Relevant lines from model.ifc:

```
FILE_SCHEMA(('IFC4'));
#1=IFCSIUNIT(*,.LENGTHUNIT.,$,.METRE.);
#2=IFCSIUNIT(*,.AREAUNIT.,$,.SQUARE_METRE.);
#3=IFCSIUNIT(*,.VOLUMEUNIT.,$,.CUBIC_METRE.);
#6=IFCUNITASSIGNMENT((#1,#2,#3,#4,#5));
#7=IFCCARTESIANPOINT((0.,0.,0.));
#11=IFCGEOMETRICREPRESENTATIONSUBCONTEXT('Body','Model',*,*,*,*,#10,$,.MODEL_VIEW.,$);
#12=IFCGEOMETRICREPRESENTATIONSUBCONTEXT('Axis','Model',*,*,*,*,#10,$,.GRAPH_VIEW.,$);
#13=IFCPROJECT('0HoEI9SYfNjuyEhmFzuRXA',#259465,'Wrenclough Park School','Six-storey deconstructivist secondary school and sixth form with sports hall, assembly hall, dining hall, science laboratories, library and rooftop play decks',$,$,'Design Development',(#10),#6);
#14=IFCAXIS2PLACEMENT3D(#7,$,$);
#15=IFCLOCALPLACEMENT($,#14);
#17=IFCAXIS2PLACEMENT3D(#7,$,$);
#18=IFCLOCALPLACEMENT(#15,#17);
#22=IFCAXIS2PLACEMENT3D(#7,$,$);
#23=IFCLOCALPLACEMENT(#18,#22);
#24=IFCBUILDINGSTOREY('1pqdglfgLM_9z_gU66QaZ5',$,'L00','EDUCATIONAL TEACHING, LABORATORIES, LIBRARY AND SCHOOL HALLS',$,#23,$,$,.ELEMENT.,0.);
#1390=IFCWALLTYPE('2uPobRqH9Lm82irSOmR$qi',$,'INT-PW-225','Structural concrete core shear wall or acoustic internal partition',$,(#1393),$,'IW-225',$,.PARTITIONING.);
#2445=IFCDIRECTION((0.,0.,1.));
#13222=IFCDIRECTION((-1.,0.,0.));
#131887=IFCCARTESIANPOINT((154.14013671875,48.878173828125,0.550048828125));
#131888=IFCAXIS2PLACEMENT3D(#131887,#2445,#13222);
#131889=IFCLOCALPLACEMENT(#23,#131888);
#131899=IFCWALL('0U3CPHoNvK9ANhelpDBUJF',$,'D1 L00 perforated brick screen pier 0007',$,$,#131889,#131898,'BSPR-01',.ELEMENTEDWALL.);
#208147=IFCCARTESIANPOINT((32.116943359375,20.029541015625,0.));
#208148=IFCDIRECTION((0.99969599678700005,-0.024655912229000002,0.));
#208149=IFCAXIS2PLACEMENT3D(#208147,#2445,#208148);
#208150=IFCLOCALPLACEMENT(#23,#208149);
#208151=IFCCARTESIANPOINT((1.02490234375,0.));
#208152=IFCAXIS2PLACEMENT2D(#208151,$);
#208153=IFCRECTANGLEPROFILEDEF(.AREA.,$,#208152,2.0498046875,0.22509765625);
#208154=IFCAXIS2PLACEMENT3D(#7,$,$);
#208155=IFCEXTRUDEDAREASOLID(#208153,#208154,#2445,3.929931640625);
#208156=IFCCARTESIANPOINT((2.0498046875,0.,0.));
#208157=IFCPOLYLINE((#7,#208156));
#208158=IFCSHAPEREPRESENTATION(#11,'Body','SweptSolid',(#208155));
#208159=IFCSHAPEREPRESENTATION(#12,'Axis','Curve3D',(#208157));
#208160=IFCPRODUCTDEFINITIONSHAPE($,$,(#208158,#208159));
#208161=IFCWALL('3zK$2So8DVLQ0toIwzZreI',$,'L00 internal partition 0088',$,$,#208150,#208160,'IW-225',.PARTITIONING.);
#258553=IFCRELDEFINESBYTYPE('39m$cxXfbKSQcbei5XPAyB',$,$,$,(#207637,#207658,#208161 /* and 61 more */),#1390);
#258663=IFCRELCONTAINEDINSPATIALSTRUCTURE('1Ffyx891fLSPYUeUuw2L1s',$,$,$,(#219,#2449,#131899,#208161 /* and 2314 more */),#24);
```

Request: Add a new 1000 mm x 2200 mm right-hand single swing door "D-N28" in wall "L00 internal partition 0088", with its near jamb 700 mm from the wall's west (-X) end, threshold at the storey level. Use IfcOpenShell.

```python
import numpy as np
import ifcopenshell
import ifcopenshell.api.feature
import ifcopenshell.api.geometry
import ifcopenshell.api.root
import ifcopenshell.api.spatial
import ifcopenshell.geom
import ifcopenshell.util.element
import ifcopenshell.util.placement
import ifcopenshell.util.representation
import ifcopenshell.util.shape
import ifcopenshell.util.unit

model = ifcopenshell.open("model.ifc")
unit_scale = ifcopenshell.util.unit.calculate_unit_scale(model)
settings = ifcopenshell.geom.settings()


def volume(element):
    """Net volume in cubic metres, openings subtracted."""
    shape = ifcopenshell.geom.create_shape(settings, element)
    return ifcopenshell.util.shape.get_volume(shape.geometry)


wall = model.by_guid("3zK$2So8DVLQ0toIwzZreI")
storey = ifcopenshell.util.element.get_container(wall, ifc_class="IfcBuildingStorey")
context = ifcopenshell.util.representation.get_context(model, "Model", "Body", "MODEL_VIEW")
before = volume(wall)

width, height, from_end, sill = 1, 2.2, 0.7, 0.0  # metres

# The wall runs along its own X axis, and the end named is its -X end.
wall_shape = ifcopenshell.geom.create_shape(settings, wall)
x, y, z = ifcopenshell.util.shape.get_vertices(wall_shape.geometry).T
start = x.min() + from_end
face, thickness = float(y.min()), float(y.max() - y.min())
wall_matrix = ifcopenshell.util.placement.get_local_placement(wall.ObjectPlacement)
level = ifcopenshell.util.placement.get_local_placement(storey.ObjectPlacement)[2, 3]


def in_wall(x, y):
    """Placement at x, y metres in the wall's axes, at sill height."""
    matrix = wall_matrix.copy()
    matrix[:, 3] = wall_matrix @ np.array([x / unit_scale, y / unit_scale, 0.0, 1.0])
    matrix[2, 3] = level + sill / unit_scale
    return matrix


# Opening: a box that overshoots both wall faces by 50 mm.
opening = ifcopenshell.api.root.create_entity(model, ifc_class="IfcOpeningElement", predefined_type="OPENING")
box = ifcopenshell.api.geometry.add_wall_representation(
    model, context=context, length=width, height=height, thickness=thickness + 0.1
)
ifcopenshell.api.geometry.assign_representation(model, product=opening, representation=box)
ifcopenshell.api.geometry.edit_object_placement(model, product=opening, matrix=in_wall(start, face - 0.05), is_si=False)
ifcopenshell.api.feature.add_feature(model, feature=opening, element=wall)

door = ifcopenshell.api.root.create_entity(model, ifc_class="IfcDoor", name="D-N28", predefined_type="DOOR")
door.OverallWidth, door.OverallHeight = width / unit_scale, height / unit_scale
door.OperationType = "SINGLE_SWING_RIGHT"
body = ifcopenshell.api.geometry.add_door_representation(
    model,
    context=context,
    overall_width=door.OverallWidth,
    overall_height=door.OverallHeight,
    operation_type="SINGLE_SWING_RIGHT",
    lining_properties={"LiningDepth": thickness / unit_scale, "ThresholdDepth": thickness / unit_scale},
)
ifcopenshell.api.geometry.assign_representation(model, product=door, representation=body)
ifcopenshell.api.spatial.assign_container(model, products=[door], relating_structure=storey)
ifcopenshell.api.feature.add_filling(model, opening=opening, element=door)

# The lining spans the wall, so the door starts at the wall face.
ifcopenshell.api.geometry.edit_object_placement(model, product=door, matrix=in_wall(start, face), is_si=False)

after = volume(wall)

print(f"wall volume {before:.3f} -> {after:.3f} m3")

model.write("model_v2.ifc")
```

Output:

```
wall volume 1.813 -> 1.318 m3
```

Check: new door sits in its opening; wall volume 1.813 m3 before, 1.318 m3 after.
